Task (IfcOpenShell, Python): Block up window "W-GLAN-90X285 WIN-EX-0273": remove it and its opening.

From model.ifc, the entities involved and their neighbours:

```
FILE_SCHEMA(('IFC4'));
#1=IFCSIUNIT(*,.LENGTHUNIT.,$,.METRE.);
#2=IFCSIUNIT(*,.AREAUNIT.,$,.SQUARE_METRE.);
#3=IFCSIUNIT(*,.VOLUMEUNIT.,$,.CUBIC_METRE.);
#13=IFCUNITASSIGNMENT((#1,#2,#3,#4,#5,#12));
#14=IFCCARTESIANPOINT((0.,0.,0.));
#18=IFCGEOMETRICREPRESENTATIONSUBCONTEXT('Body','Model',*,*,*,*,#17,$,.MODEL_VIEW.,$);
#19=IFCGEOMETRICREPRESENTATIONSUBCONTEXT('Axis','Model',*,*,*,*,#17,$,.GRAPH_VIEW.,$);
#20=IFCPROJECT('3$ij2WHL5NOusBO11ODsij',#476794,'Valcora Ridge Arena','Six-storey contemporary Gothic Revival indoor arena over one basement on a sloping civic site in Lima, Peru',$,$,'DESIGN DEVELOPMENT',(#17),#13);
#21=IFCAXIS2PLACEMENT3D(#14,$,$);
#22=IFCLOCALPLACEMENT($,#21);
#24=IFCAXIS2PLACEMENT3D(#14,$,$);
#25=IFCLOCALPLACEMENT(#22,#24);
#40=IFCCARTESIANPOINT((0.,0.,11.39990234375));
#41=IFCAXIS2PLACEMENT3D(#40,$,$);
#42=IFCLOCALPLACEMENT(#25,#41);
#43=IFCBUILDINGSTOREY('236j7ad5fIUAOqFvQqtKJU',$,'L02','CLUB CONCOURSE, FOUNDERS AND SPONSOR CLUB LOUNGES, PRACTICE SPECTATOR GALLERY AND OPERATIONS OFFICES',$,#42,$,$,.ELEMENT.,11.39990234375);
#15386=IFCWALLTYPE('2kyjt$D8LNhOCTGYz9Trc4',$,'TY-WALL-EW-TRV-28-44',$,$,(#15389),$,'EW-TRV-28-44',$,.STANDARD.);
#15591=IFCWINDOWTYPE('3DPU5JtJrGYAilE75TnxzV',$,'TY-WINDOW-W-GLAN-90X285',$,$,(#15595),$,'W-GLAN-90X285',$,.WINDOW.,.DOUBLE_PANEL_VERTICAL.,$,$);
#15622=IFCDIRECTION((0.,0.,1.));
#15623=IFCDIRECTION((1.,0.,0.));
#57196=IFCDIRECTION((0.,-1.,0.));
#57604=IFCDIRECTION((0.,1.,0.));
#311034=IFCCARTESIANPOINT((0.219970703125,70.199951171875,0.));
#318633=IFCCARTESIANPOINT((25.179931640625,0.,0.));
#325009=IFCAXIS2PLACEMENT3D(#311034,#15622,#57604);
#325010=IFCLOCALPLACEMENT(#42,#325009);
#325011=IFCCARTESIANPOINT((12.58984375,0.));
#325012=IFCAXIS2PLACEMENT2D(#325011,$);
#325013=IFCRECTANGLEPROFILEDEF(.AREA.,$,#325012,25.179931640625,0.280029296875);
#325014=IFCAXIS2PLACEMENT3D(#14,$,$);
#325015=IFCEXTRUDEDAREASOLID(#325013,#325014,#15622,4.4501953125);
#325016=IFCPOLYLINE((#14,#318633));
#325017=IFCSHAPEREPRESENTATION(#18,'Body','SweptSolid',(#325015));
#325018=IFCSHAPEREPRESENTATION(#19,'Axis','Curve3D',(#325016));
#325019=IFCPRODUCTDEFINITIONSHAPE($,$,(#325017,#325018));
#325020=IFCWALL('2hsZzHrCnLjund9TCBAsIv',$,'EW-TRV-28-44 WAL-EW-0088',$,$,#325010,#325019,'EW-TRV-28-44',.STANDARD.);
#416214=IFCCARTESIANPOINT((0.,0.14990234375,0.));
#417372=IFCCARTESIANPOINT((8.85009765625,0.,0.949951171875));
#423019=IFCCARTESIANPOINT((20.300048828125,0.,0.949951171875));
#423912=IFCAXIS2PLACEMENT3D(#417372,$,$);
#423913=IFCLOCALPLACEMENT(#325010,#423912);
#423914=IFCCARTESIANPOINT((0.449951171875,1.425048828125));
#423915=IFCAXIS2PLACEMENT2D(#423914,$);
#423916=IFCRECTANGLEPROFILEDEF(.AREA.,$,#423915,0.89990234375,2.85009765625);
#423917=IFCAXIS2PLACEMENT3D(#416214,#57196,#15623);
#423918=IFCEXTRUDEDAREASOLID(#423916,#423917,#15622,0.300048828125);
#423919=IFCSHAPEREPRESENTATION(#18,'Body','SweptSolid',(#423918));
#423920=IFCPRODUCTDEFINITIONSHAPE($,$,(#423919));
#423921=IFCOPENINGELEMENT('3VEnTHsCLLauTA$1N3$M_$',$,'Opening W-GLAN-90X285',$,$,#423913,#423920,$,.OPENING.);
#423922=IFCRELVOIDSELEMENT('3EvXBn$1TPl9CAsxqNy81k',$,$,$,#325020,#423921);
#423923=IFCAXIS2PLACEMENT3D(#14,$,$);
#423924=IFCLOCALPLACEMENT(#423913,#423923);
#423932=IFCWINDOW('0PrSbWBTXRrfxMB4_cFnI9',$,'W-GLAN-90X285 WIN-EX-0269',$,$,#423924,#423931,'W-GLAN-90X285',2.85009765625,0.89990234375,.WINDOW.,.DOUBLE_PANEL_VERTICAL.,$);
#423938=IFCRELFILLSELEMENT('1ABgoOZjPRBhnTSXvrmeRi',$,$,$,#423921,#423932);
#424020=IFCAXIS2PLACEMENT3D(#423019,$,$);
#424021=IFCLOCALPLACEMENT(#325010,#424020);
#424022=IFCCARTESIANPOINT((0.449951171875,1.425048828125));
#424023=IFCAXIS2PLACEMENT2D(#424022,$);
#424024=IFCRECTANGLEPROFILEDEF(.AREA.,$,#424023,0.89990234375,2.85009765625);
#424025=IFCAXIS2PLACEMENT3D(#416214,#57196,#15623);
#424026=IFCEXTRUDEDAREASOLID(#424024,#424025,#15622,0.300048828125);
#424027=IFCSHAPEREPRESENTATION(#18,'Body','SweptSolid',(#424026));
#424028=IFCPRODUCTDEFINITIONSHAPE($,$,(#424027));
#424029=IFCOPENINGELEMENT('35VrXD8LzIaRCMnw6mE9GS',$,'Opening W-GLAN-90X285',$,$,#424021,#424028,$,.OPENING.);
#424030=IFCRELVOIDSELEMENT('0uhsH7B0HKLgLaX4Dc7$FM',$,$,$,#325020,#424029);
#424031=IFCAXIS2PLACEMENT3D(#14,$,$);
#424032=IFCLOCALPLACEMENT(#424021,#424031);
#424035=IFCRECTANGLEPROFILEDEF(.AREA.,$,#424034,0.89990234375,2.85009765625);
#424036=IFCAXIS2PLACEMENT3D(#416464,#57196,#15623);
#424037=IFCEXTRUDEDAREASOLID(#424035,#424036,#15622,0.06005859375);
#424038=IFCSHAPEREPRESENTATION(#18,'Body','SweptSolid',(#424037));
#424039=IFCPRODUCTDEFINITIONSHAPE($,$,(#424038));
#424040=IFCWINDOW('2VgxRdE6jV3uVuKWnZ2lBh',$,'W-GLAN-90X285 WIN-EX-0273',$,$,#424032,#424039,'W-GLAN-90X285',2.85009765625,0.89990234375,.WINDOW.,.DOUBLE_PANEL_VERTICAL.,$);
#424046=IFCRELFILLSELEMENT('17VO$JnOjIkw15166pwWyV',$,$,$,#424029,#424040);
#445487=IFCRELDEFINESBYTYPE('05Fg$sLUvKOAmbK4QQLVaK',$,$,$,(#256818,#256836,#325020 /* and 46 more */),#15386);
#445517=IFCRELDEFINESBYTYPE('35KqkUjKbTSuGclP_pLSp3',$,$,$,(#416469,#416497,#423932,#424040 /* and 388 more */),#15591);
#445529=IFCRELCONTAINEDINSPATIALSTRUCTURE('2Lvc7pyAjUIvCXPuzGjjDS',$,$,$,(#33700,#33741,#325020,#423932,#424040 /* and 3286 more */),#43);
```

```python
import ifcopenshell
import ifcopenshell.api.feature
import ifcopenshell.api.root
import ifcopenshell.geom
import ifcopenshell.util.shape

model = ifcopenshell.open("model.ifc")
settings = ifcopenshell.geom.settings()


def volume(element):
    """Net volume in cubic metres, openings subtracted."""
    shape = ifcopenshell.geom.create_shape(settings, element)
    return ifcopenshell.util.shape.get_volume(shape.geometry)


window = model.by_id(424040)
opening = window.FillsVoids[0].RelatingOpeningElement
wall = opening.VoidsElements[0].RelatingBuildingElement
before = volume(wall)

ifcopenshell.api.root.remove_product(model, product=window)
ifcopenshell.api.feature.remove_feature(model, feature=opening)

after = volume(wall)

print(f"wall volume {before:.3f} -> {after:.3f} m3")

model.write("model_rev.ifc")
```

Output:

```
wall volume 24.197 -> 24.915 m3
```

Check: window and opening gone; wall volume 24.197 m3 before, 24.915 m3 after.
